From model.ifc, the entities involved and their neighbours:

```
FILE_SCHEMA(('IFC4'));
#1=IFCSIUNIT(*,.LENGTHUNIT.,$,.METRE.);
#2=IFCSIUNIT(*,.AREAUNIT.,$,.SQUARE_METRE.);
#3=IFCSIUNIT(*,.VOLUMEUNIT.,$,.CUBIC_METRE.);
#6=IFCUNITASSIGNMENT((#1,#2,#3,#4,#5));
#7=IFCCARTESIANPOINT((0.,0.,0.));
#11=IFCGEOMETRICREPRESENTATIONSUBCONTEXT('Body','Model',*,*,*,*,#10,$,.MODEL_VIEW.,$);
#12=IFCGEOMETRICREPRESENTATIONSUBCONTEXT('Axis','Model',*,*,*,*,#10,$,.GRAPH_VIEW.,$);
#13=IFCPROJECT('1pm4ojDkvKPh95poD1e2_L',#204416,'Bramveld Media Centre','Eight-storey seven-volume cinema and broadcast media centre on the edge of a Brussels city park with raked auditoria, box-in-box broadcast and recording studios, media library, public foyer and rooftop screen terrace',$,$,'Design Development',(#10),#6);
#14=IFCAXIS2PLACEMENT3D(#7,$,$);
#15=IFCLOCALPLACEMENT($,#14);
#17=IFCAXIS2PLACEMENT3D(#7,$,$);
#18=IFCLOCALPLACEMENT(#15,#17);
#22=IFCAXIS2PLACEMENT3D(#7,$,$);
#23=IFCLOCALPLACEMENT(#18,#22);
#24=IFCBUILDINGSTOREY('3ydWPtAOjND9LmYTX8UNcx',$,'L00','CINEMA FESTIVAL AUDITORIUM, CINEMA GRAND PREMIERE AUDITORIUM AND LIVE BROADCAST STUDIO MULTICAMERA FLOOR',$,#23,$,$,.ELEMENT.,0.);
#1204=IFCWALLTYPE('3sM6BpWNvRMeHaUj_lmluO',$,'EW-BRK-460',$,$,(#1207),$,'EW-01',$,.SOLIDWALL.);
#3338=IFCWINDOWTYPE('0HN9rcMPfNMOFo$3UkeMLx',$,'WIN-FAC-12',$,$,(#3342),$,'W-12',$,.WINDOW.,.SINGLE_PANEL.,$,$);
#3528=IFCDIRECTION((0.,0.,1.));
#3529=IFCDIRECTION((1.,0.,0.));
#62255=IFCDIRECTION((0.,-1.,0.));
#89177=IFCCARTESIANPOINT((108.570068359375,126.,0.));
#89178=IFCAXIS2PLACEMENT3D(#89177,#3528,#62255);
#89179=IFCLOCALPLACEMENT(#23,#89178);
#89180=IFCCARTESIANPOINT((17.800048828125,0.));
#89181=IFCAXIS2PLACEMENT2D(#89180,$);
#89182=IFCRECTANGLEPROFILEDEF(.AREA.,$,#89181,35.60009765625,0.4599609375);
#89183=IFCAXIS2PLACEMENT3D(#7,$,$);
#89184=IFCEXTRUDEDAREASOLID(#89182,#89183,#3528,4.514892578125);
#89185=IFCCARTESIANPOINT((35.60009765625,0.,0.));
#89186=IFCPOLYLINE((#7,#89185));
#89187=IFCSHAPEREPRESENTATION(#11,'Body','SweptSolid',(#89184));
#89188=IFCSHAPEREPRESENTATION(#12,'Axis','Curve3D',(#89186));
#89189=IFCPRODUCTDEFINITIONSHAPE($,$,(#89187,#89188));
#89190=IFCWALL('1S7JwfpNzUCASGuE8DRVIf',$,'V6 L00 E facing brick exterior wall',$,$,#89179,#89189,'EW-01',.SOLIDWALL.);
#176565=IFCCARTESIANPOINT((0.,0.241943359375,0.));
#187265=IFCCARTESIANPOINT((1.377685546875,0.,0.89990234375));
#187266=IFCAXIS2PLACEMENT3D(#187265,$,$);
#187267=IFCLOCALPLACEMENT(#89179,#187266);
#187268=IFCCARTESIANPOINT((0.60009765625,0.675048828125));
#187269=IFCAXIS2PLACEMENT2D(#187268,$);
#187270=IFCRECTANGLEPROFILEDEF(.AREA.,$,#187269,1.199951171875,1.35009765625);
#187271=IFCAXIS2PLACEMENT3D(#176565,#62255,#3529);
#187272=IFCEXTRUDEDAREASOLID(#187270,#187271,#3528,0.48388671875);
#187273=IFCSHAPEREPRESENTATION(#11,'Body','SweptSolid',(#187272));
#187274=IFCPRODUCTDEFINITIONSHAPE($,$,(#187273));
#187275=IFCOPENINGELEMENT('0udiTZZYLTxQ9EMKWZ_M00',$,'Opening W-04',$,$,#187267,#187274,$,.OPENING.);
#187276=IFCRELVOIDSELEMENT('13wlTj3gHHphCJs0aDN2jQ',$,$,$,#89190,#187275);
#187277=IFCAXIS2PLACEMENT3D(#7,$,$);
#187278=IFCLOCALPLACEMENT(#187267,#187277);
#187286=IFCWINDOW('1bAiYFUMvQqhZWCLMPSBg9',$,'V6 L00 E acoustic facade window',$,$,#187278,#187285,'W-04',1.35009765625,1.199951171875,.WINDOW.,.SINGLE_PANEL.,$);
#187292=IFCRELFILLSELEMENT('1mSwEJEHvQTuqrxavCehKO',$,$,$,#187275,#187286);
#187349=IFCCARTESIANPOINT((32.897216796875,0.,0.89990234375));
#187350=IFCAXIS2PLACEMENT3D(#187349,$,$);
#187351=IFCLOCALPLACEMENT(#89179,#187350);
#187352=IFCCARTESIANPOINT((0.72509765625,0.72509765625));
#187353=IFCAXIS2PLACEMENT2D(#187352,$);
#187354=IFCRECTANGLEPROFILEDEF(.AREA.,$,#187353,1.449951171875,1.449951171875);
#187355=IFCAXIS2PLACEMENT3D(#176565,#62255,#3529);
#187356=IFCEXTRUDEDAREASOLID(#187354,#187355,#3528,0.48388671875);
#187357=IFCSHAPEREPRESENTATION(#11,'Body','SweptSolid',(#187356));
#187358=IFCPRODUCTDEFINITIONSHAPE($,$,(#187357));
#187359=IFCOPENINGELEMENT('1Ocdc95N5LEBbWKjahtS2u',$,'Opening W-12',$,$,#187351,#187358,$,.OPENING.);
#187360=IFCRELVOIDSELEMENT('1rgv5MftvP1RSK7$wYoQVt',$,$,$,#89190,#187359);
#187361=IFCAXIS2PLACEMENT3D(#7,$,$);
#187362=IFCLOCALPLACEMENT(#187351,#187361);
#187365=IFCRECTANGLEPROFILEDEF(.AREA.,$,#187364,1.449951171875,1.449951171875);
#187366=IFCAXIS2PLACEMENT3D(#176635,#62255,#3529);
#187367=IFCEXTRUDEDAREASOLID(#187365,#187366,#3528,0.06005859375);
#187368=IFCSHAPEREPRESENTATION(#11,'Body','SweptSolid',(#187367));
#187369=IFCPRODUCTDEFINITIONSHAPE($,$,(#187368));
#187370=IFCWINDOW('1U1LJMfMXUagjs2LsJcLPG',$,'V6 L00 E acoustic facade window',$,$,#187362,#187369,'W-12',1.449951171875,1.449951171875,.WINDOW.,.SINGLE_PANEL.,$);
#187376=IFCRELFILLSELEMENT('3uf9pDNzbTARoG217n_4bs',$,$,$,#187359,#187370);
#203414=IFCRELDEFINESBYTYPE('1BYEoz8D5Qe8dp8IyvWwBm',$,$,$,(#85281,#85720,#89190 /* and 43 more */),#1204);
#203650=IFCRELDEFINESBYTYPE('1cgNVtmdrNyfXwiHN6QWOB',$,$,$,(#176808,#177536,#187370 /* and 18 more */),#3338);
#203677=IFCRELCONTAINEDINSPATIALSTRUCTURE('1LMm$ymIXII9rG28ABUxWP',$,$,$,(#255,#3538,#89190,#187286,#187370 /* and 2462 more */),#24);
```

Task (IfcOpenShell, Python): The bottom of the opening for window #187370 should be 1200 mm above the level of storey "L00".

```python
import numpy as np
import ifcopenshell
import ifcopenshell.api.geometry
import ifcopenshell.geom
import ifcopenshell.util.element
import ifcopenshell.util.placement
import ifcopenshell.util.shape
import ifcopenshell.util.unit

model = ifcopenshell.open("model.ifc")
unit_scale = ifcopenshell.util.unit.calculate_unit_scale(model)

window = model.by_id(187370)
opening = window.FillsVoids[0].RelatingOpeningElement
storey = ifcopenshell.util.element.get_container(window, ifc_class="IfcBuildingStorey")
level = ifcopenshell.util.placement.get_local_placement(storey.ObjectPlacement)[2, 3]

# The opening's origin need not be at the sill, so measure its lowest point.
shape = ifcopenshell.geom.create_shape(ifcopenshell.geom.settings(), opening)
bottom = ifcopenshell.util.shape.get_shape_bottom_elevation(shape, shape.geometry) / unit_scale
dz = level + 1.2 / unit_scale - bottom

shift = np.array([0.0, 0.0, dz])
# The window is placed relative to its opening, so it follows when the opening moves.
matrix = ifcopenshell.util.placement.get_local_placement(opening.ObjectPlacement)
matrix[:3, 3] += shift
ifcopenshell.api.geometry.edit_object_placement(
    model, product=opening, matrix=matrix, is_si=False, should_transform_children=True
)

print(f"moved by {dz * unit_scale:+.3f} m")

model.write("model-out.ifc")
```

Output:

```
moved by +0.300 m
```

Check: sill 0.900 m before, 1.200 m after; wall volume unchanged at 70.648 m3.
